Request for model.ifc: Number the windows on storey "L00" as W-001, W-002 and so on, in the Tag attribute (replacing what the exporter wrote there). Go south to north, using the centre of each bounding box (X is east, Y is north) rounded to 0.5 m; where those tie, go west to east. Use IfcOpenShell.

First a look at what the model holds.

```python
import ifcopenshell
import ifcopenshell.util.element
import ifcopenshell.util.placement

model = ifcopenshell.open("model.ifc")
print(model.schema)
storey = next(s for s in model.by_type("IfcBuildingStorey") if s.Name == "L00")
windows = [e for e in ifcopenshell.util.element.get_decomposition(storey) if e.is_a("IfcWindow")]
for e in sorted(windows, key=lambda e: e.id()):
    origin = ifcopenshell.util.placement.get_local_placement(e.ObjectPlacement)[:3, 3]
    print(e.id(), e.Tag, e.Name, origin.round(2) + 0.0, sep=" | ")
```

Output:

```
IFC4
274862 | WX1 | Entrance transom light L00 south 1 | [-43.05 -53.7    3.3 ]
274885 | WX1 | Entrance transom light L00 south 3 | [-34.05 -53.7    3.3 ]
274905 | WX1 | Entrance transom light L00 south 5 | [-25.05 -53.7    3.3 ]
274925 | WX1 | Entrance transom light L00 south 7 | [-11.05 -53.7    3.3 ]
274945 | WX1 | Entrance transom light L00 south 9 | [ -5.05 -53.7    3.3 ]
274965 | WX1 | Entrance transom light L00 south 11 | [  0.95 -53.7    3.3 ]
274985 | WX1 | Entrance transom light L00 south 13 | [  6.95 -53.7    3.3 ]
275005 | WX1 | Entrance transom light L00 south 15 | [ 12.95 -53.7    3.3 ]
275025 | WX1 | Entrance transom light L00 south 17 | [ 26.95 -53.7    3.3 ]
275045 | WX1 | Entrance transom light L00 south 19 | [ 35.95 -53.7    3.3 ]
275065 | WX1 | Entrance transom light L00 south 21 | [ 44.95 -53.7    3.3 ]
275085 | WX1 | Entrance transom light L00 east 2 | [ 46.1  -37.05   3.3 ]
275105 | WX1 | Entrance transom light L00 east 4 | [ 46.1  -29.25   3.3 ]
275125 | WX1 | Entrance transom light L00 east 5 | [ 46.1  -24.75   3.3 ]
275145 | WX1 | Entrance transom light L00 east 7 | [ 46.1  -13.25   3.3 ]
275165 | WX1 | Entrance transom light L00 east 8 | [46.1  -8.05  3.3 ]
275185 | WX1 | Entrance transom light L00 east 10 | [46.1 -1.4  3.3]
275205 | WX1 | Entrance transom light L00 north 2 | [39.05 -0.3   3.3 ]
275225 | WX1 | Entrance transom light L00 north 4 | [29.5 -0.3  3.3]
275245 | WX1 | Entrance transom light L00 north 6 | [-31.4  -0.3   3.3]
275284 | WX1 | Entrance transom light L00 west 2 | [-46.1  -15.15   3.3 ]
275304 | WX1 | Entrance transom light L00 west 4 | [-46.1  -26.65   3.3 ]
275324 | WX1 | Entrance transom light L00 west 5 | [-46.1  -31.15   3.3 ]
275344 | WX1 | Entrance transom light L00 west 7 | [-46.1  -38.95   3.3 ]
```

```python
import ifcopenshell
import ifcopenshell.geom
import ifcopenshell.util.element
import ifcopenshell.util.shape

model = ifcopenshell.open("model.ifc")
settings = ifcopenshell.geom.settings()
settings.set("use-world-coords", True)


def centre(element):
    shape = ifcopenshell.geom.create_shape(settings, element)
    return ifcopenshell.util.shape.get_bbox_centroid(shape.geometry)


storey = next(s for s in model.by_type("IfcBuildingStorey") if s.Name == "L00")
windows = [e for e in ifcopenshell.util.element.get_decomposition(storey) if e.is_a("IfcWindow")]

# Insertion points can sit at a corner or the storey origin, so sort by the geometry (in metres).
centres = {e: centre(e) for e in windows}
windows.sort(key=lambda e: (round(centres[e][1] / 0.5), centres[e][0]))

for i, e in enumerate(windows, start=1):
    number = f"W-0{i:02d}"
    e.Tag = number
    print(e.id(), number)

model.write("model_updated.ifc")
```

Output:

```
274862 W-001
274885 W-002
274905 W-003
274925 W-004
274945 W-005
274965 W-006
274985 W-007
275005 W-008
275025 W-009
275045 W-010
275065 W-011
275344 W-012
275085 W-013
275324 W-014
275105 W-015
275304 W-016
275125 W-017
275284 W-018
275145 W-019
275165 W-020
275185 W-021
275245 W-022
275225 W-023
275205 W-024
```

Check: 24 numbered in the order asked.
